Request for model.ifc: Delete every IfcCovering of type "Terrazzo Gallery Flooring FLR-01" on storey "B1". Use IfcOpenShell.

First a look at what the model holds.

```python
import ifcopenshell
import ifcopenshell.util.element

model = ifcopenshell.open("model.ifc")
print(model.schema)
storey = next(s for s in model.by_type("IfcBuildingStorey") if s.Name == "B1")
coverings = [e for e in ifcopenshell.util.element.get_decomposition(storey) if e.is_a("IfcCovering")]
seen = {}
for e in coverings:
    element_type = ifcopenshell.util.element.get_type(e)
    name = element_type.Name if element_type not in (None, e) else None
    seen[name] = seen.get(name, 0) + 1
for name, count in sorted(seen.items(), key=str):
    print(count, "x", name)
```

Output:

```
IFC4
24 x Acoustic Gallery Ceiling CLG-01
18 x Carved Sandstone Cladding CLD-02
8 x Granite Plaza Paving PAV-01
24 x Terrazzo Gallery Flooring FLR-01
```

```python
import ifcopenshell
import ifcopenshell.api.root
import ifcopenshell.util.element

model = ifcopenshell.open("model.ifc")

storey = next(s for s in model.by_type("IfcBuildingStorey") if s.Name == "B1")
coverings = [e for e in ifcopenshell.util.element.get_decomposition(storey) if e.is_a("IfcCovering")]
targets = [e for e in coverings if (t := ifcopenshell.util.element.get_type(e)) not in (None, e) and t.Name == "Terrazzo Gallery Flooring FLR-01"]

for e in targets:
    ifcopenshell.api.root.remove_product(model, product=e)
print(len(targets), "removed")

model.write("model_rev.ifc")
```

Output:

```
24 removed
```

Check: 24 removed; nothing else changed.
